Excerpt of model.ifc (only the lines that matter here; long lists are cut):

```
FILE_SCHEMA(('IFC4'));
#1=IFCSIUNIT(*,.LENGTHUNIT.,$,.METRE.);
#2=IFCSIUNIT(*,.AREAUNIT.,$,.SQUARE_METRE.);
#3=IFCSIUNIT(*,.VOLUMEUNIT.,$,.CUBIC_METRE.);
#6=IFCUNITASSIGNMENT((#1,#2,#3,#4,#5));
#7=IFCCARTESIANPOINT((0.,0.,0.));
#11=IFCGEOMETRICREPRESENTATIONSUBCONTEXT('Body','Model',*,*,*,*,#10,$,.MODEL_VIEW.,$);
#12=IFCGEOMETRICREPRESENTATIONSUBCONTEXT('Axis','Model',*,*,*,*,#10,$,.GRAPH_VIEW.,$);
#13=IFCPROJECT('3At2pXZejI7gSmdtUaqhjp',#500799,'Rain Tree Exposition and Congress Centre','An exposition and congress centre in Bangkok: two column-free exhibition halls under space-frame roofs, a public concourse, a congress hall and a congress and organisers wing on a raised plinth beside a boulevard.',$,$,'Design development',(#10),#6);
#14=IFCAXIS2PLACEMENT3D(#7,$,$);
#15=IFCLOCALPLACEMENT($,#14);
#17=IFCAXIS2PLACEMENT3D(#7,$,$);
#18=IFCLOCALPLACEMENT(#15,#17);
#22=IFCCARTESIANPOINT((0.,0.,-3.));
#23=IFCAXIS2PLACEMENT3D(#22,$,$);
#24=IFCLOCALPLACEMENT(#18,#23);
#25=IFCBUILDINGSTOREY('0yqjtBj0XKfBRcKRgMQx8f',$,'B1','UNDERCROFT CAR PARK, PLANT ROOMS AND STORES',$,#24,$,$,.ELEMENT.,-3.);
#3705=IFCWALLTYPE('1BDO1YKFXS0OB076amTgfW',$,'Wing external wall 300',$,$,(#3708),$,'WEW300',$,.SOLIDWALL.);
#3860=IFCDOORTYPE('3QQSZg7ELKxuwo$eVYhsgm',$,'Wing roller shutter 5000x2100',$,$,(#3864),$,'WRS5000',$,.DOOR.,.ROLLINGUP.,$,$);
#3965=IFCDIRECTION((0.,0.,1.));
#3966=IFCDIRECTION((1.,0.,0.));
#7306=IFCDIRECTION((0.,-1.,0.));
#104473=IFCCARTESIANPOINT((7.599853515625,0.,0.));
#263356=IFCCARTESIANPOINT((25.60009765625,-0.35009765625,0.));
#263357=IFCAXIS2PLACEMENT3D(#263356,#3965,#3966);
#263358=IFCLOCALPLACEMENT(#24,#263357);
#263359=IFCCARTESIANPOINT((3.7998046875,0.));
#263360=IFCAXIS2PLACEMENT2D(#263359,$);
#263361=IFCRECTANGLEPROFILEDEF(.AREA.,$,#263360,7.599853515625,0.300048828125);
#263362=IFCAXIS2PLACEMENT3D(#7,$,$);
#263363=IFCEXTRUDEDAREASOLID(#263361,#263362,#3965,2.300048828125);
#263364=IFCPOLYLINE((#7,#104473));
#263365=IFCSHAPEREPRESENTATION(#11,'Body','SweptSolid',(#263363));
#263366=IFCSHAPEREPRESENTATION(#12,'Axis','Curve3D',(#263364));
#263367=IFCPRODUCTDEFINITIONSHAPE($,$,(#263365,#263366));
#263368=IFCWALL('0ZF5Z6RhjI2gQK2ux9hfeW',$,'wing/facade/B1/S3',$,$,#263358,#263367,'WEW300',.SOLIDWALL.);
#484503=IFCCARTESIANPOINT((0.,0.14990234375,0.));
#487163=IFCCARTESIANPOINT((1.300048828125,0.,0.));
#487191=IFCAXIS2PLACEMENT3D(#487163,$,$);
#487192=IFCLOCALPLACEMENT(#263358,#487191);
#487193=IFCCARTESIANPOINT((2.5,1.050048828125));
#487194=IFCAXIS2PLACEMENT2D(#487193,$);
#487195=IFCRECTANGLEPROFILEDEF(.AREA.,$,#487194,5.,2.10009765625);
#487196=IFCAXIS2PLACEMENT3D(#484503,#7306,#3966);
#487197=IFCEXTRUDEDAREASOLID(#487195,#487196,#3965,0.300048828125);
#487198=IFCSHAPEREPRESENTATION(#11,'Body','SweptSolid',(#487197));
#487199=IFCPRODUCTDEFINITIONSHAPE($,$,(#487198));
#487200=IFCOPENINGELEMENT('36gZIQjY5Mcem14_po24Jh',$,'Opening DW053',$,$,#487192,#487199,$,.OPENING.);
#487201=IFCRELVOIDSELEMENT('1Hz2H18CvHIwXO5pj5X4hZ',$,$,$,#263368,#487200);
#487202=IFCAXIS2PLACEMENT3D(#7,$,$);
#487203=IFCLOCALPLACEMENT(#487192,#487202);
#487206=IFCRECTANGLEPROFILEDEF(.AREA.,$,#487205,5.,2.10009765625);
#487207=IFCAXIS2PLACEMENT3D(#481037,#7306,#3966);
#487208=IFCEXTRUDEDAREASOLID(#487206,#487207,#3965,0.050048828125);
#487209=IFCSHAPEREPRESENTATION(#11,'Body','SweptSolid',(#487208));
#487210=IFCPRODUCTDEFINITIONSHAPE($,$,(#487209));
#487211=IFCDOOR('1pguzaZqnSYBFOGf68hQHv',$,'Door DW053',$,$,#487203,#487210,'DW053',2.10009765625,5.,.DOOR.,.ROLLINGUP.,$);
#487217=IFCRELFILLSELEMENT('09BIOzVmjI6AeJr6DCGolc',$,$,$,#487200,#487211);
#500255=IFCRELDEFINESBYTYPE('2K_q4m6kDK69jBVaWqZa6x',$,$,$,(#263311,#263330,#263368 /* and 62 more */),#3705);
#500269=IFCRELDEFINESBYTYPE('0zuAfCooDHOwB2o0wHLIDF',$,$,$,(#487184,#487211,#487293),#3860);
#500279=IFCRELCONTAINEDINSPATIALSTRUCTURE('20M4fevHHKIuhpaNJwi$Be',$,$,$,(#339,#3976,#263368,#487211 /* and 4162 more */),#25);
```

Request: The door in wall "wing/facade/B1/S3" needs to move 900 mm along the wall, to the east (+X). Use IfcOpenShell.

```python
import ifcopenshell
import ifcopenshell.api.geometry
import ifcopenshell.util.placement

model = ifcopenshell.open("model.ifc")

door = model.by_guid("1pguzaZqnSYBFOGf68hQHv")
opening = door.FillsVoids[0].RelatingOpeningElement
wall = opening.VoidsElements[0].RelatingBuildingElement

wall_matrix = ifcopenshell.util.placement.get_local_placement(wall.ObjectPlacement)
shift = wall_matrix[:3, 0] * 0.9
before = ifcopenshell.util.placement.get_local_placement(door.ObjectPlacement)[:3, 3].copy()

# The door is placed relative to its opening, so it follows when the opening moves.
matrix = ifcopenshell.util.placement.get_local_placement(opening.ObjectPlacement)
matrix[:3, 3] += shift
ifcopenshell.api.geometry.edit_object_placement(
    model, product=opening, matrix=matrix, is_si=False, should_transform_children=True
)

after = ifcopenshell.util.placement.get_local_placement(door.ObjectPlacement)[:3, 3]
print("door moved by", (after - before).round(3) + 0.0)

model.write("model_rev.ifc")
```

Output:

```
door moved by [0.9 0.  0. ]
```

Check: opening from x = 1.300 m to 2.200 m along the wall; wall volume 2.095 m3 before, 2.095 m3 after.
